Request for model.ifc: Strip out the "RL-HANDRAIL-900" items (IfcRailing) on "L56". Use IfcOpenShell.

First a look at what the model holds.

```python
import ifcopenshell
import ifcopenshell.util.element

model = ifcopenshell.open("model.ifc")
print(model.schema)
storey = next(s for s in model.by_type("IfcBuildingStorey") if s.Name == "L56")
railings = [e for e in ifcopenshell.util.element.get_decomposition(storey) if e.is_a("IfcRailing")]
seen = {}
for e in railings:
    element_type = ifcopenshell.util.element.get_type(e)
    name = element_type.Name if element_type not in (None, e) else None
    seen[name] = seen.get(name, 0) + 1
for name, count in sorted(seen.items(), key=str):
    print(count, "x", name)
```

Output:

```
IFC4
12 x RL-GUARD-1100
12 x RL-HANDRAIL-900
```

```python
import ifcopenshell
import ifcopenshell.api.root
import ifcopenshell.util.element

model = ifcopenshell.open("model.ifc")

storey = next(s for s in model.by_type("IfcBuildingStorey") if s.Name == "L56")
railings = [e for e in ifcopenshell.util.element.get_decomposition(storey) if e.is_a("IfcRailing")]
targets = [e for e in railings if (t := ifcopenshell.util.element.get_type(e)) not in (None, e) and t.Name == "RL-HANDRAIL-900"]

for e in targets:
    ifcopenshell.api.root.remove_product(model, product=e)
print(len(targets), "removed")

model.write("model_updated.ifc")
```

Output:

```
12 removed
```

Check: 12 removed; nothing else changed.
